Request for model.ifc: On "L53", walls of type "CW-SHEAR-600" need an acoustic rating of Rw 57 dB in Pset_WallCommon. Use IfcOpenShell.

First a look at what the model holds.

```python
import ifcopenshell
import ifcopenshell.util.element

model = ifcopenshell.open("model.ifc")
print(model.schema)
storey = next(s for s in model.by_type("IfcBuildingStorey") if s.Name == "L53")
walls = [e for e in ifcopenshell.util.element.get_decomposition(storey) if e.is_a("IfcWall")]
seen = {}
for e in walls:
    element_type = ifcopenshell.util.element.get_type(e)
    key = (element_type.Name if element_type != e and element_type else None, ifcopenshell.util.element.get_pset(e, "Pset_WallCommon", "AcousticRating"))
    seen[key] = seen.get(key, 0) + 1
for (name, value), count in sorted(seen.items(), key=str):
    print(count, "x", name, "|", value)
```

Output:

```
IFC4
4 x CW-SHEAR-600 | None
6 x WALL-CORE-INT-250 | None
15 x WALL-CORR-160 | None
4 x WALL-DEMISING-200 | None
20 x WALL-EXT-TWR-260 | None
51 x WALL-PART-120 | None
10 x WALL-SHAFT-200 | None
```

```python
import ifcopenshell
import ifcopenshell.api.pset
import ifcopenshell.util.element

model = ifcopenshell.open("model.ifc")

storey = next(s for s in model.by_type("IfcBuildingStorey") if s.Name == "L53")
walls = [e for e in ifcopenshell.util.element.get_decomposition(storey) if e.is_a("IfcWall")]

count = 0
for e in walls:
    element_type = ifcopenshell.util.element.get_type(e)
    if element_type in (None, e) or element_type.Name != "CW-SHEAR-600":
        continue
    found = ifcopenshell.util.element.get_pset(e, "Pset_WallCommon", should_inherit=False)
    if found:
        pset = model.by_id(found["id"])
        if len(ifcopenshell.util.element.get_elements_by_pset(pset)) > 1:
            pset = ifcopenshell.api.pset.unshare_pset(model, products=[e], pset=pset)[0]
    else:
        pset = ifcopenshell.api.pset.add_pset(model, product=e, name="Pset_WallCommon")
    ifcopenshell.api.pset.edit_pset(model, pset=pset, properties={"AcousticRating": "Rw 57 dB"})
    count += 1

print(count, "walls updated")

model.write("model_rev.ifc")
```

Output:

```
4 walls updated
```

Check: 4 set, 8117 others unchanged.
